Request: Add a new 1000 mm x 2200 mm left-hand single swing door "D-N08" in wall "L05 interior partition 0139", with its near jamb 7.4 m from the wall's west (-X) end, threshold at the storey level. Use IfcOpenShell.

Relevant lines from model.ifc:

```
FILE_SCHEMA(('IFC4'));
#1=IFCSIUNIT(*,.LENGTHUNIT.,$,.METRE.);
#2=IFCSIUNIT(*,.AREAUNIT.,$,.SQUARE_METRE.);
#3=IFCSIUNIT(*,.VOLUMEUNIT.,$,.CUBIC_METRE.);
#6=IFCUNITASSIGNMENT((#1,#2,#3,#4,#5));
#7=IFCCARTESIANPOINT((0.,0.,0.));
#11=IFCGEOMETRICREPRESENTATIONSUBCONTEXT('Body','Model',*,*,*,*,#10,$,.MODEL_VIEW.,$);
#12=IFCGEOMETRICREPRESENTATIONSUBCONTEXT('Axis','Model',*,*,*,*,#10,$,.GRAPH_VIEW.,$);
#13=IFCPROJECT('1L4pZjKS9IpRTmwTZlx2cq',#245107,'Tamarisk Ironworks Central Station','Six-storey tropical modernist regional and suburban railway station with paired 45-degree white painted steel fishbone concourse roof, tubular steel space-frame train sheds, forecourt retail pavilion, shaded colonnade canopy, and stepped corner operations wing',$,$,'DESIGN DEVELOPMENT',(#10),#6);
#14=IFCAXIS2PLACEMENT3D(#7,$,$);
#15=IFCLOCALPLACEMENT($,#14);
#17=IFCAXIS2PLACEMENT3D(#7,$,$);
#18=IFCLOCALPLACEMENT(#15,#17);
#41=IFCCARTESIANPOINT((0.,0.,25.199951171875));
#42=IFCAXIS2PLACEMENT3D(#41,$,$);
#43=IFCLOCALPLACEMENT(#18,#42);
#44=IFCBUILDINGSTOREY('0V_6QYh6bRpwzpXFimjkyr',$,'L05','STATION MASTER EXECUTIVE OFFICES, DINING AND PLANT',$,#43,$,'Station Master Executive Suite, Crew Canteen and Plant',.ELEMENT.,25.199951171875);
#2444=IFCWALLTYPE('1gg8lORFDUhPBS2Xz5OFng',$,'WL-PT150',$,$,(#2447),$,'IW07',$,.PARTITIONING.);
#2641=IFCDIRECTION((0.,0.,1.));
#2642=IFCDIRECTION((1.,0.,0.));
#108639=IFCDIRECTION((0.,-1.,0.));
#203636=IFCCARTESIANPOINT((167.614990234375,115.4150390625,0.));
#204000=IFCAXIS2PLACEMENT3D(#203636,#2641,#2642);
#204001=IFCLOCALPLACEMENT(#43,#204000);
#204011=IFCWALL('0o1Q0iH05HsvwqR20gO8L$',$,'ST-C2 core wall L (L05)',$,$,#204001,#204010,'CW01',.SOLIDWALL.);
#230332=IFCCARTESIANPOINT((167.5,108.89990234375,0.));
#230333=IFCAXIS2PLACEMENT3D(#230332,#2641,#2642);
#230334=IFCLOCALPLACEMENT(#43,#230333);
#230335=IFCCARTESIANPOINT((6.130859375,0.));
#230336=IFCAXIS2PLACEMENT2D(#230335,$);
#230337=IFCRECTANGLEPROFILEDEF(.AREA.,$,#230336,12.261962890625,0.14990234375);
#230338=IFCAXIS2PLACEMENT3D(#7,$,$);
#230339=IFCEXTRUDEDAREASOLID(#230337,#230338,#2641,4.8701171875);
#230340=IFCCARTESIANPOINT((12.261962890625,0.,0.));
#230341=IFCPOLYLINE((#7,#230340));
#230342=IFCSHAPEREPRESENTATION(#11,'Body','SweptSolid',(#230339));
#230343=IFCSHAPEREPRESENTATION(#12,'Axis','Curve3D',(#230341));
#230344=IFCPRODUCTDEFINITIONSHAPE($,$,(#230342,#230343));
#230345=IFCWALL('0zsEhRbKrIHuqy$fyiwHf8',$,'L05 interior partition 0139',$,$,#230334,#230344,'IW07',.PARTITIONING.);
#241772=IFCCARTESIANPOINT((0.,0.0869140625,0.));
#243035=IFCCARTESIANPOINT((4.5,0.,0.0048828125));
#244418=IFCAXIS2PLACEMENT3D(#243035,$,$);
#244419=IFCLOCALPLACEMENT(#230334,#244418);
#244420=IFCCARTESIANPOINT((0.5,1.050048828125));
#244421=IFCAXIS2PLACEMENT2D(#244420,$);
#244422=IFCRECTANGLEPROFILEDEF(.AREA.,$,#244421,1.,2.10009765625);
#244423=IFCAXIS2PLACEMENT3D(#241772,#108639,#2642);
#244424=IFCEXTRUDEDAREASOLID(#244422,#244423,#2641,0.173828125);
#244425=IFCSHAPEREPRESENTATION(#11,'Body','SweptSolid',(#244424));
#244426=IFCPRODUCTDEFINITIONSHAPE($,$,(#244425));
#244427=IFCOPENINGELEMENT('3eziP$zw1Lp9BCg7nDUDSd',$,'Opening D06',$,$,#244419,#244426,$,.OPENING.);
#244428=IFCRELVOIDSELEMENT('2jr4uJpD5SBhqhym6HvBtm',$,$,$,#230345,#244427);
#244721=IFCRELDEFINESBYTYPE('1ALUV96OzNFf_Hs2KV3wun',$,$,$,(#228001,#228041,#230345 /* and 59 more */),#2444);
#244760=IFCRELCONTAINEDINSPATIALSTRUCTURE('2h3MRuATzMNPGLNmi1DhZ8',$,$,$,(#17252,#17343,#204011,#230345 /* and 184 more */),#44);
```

```python
import numpy as np
import ifcopenshell
import ifcopenshell.api.feature
import ifcopenshell.api.geometry
import ifcopenshell.api.root
import ifcopenshell.api.spatial
import ifcopenshell.geom
import ifcopenshell.util.element
import ifcopenshell.util.placement
import ifcopenshell.util.representation
import ifcopenshell.util.shape
import ifcopenshell.util.unit

model = ifcopenshell.open("model.ifc")
unit_scale = ifcopenshell.util.unit.calculate_unit_scale(model)
settings = ifcopenshell.geom.settings()


def volume(element):
    """Net volume in cubic metres, openings subtracted."""
    shape = ifcopenshell.geom.create_shape(settings, element)
    return ifcopenshell.util.shape.get_volume(shape.geometry)


wall = model.by_id(230345)
storey = ifcopenshell.util.element.get_container(wall, ifc_class="IfcBuildingStorey")
context = ifcopenshell.util.representation.get_context(model, "Model", "Body", "MODEL_VIEW")
before = volume(wall)

width, height, from_end, sill = 1, 2.2, 7.4, 0.0  # metres

# The wall runs along its own X axis, and the end named is its -X end.
wall_shape = ifcopenshell.geom.create_shape(settings, wall)
x, y, z = ifcopenshell.util.shape.get_vertices(wall_shape.geometry).T
start = x.min() + from_end
face, thickness = float(y.min()), float(y.max() - y.min())
wall_matrix = ifcopenshell.util.placement.get_local_placement(wall.ObjectPlacement)
level = ifcopenshell.util.placement.get_local_placement(storey.ObjectPlacement)[2, 3]


def in_wall(x, y):
    """Placement at x, y metres in the wall's axes, at sill height."""
    matrix = wall_matrix.copy()
    matrix[:, 3] = wall_matrix @ np.array([x / unit_scale, y / unit_scale, 0.0, 1.0])
    matrix[2, 3] = level + sill / unit_scale
    return matrix


# Opening: a box that overshoots both wall faces by 50 mm.
opening = ifcopenshell.api.root.create_entity(model, ifc_class="IfcOpeningElement", predefined_type="OPENING")
box = ifcopenshell.api.geometry.add_wall_representation(
    model, context=context, length=width, height=height, thickness=thickness + 0.1
)
ifcopenshell.api.geometry.assign_representation(model, product=opening, representation=box)
ifcopenshell.api.geometry.edit_object_placement(model, product=opening, matrix=in_wall(start, face - 0.05), is_si=False)
ifcopenshell.api.feature.add_feature(model, feature=opening, element=wall)

door = ifcopenshell.api.root.create_entity(model, ifc_class="IfcDoor", name="D-N08", predefined_type="DOOR")
door.OverallWidth, door.OverallHeight = width / unit_scale, height / unit_scale
door.OperationType = "SINGLE_SWING_LEFT"
body = ifcopenshell.api.geometry.add_door_representation(
    model,
    context=context,
    overall_width=door.OverallWidth,
    overall_height=door.OverallHeight,
    operation_type="SINGLE_SWING_LEFT",
    lining_properties={"LiningDepth": thickness / unit_scale, "ThresholdDepth": thickness / unit_scale},
)
ifcopenshell.api.geometry.assign_representation(model, product=door, representation=body)
ifcopenshell.api.spatial.assign_container(model, products=[door], relating_structure=storey)
ifcopenshell.api.feature.add_filling(model, opening=opening, element=door)

# The lining spans the wall, so the door starts at the wall face.
ifcopenshell.api.geometry.edit_object_placement(model, product=door, matrix=in_wall(start, face), is_si=False)

after = volume(wall)

print(f"wall volume {before:.3f} -> {after:.3f} m3")

model.write("model_edited.ifc")
```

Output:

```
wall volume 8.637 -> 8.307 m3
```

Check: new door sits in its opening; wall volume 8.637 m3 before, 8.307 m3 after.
